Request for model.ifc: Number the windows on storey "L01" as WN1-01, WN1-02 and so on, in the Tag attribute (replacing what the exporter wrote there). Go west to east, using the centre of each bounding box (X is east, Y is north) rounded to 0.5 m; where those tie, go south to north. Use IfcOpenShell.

First a look at what the model holds.

```python
import ifcopenshell
import ifcopenshell.util.element
import ifcopenshell.util.placement

model = ifcopenshell.open("model.ifc")
print(model.schema)
storey = next(s for s in model.by_type("IfcBuildingStorey") if s.Name == "L01")
windows = [e for e in ifcopenshell.util.element.get_decomposition(storey) if e.is_a("IfcWindow")]
for e in sorted(windows, key=lambda e: e.id()):
    origin = ifcopenshell.util.placement.get_local_placement(e.ObjectPlacement)[:3, 3]
    print(e.id(), e.Tag, e.Name, origin.round(2) + 0.0, sep=" | ")
```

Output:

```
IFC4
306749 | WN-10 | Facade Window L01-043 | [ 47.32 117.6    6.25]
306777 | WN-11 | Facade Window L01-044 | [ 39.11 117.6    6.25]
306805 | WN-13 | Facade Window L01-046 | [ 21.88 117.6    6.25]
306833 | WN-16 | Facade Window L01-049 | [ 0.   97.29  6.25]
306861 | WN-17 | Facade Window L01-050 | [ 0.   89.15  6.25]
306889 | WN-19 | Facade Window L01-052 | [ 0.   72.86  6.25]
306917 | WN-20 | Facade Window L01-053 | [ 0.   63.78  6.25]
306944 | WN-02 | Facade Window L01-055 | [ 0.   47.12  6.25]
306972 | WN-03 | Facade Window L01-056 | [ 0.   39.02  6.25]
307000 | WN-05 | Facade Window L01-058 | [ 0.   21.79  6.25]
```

```python
import ifcopenshell
import ifcopenshell.geom
import ifcopenshell.util.element
import ifcopenshell.util.shape

model = ifcopenshell.open("model.ifc")
settings = ifcopenshell.geom.settings()
settings.set("use-world-coords", True)


def centre(element):
    shape = ifcopenshell.geom.create_shape(settings, element)
    return ifcopenshell.util.shape.get_bbox_centroid(shape.geometry)


storey = next(s for s in model.by_type("IfcBuildingStorey") if s.Name == "L01")
windows = [e for e in ifcopenshell.util.element.get_decomposition(storey) if e.is_a("IfcWindow")]

# Insertion points can sit at a corner or the storey origin, so sort by the geometry (in metres).
centres = {e: centre(e) for e in windows}
windows.sort(key=lambda e: (round(centres[e][0] / 0.5), centres[e][1]))

for i, e in enumerate(windows, start=1):
    number = f"WN1-{i:02d}"
    e.Tag = number
    print(e.id(), number)

model.write("model_edited.ifc")
```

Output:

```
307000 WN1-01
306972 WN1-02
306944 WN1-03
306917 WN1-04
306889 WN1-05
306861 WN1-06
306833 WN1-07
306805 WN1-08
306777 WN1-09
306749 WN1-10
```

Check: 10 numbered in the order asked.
